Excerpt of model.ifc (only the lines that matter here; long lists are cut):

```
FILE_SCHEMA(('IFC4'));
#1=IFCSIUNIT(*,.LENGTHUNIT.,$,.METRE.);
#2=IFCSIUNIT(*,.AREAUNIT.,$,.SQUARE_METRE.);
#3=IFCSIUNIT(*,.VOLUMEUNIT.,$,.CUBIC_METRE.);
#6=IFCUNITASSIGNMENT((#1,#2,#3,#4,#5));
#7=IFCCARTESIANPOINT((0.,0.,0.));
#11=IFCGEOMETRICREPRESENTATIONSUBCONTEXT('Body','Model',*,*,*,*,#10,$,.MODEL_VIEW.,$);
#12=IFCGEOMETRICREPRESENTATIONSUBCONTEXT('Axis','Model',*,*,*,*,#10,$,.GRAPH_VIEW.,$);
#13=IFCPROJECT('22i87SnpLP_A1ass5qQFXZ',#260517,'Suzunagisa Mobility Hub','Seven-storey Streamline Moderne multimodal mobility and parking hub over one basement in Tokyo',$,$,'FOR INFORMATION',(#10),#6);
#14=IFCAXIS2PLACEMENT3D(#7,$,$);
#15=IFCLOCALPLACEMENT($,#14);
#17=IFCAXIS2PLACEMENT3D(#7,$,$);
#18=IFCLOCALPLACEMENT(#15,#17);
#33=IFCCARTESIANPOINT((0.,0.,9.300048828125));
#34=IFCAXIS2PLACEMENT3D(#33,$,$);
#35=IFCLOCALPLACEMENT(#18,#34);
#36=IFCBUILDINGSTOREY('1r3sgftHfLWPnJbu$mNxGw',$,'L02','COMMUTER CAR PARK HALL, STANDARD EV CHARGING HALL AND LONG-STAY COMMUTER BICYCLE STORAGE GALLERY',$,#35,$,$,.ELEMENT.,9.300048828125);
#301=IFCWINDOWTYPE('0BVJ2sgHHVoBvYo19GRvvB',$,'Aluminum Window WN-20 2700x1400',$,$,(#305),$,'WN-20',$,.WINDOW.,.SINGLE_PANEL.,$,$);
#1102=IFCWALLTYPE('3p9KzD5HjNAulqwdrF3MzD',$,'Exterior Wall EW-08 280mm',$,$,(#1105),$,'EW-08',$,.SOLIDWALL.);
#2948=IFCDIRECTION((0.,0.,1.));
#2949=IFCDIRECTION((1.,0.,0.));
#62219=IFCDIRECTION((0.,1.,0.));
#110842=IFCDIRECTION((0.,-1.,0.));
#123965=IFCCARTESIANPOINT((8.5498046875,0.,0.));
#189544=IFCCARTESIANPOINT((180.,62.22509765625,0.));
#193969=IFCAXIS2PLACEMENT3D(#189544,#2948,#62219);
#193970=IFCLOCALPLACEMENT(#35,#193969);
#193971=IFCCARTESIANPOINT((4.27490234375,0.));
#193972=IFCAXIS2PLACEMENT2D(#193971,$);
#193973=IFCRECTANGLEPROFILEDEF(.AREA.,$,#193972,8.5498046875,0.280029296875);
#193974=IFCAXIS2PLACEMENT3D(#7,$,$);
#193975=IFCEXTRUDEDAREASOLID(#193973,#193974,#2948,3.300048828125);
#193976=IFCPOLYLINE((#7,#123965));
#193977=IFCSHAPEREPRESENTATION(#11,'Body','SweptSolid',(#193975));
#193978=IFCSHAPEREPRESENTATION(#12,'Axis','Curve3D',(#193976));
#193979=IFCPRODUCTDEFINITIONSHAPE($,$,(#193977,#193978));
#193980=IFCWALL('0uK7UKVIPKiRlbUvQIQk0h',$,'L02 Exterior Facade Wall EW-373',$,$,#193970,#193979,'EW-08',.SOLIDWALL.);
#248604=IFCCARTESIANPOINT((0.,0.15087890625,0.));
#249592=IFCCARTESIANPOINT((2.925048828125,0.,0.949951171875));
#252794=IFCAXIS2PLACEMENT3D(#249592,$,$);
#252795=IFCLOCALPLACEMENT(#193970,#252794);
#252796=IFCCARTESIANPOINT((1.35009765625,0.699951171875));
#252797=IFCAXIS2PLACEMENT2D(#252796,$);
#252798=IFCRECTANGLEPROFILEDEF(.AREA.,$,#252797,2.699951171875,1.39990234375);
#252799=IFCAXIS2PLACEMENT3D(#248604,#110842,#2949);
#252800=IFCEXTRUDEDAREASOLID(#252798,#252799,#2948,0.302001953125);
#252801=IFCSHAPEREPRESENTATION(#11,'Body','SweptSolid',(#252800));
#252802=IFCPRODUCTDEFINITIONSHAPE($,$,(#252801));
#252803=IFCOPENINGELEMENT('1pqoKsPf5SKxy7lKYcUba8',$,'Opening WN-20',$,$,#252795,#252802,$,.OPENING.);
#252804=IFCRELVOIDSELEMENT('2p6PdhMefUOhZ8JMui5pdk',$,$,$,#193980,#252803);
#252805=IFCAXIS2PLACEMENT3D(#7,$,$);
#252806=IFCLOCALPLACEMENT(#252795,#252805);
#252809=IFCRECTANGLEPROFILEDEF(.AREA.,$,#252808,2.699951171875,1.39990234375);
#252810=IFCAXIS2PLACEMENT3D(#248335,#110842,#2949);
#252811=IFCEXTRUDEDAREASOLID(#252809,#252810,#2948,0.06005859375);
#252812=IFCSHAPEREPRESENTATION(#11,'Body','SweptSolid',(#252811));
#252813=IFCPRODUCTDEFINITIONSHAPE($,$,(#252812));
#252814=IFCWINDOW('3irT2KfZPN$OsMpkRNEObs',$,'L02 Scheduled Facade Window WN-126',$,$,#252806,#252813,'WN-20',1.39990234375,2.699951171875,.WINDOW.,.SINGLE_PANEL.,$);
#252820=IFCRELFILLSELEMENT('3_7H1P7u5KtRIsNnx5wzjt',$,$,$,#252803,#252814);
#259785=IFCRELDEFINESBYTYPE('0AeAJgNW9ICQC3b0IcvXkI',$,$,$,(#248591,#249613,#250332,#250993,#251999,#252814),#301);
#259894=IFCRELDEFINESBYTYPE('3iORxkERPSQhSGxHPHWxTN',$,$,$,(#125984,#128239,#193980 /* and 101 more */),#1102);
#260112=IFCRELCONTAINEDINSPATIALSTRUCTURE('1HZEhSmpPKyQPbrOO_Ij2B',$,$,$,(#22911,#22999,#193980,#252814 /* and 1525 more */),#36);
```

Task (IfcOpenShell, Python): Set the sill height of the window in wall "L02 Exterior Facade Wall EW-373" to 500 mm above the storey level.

```python
import numpy as np
import ifcopenshell
import ifcopenshell.api.geometry
import ifcopenshell.geom
import ifcopenshell.util.element
import ifcopenshell.util.placement
import ifcopenshell.util.shape
import ifcopenshell.util.unit

model = ifcopenshell.open("model.ifc")
unit_scale = ifcopenshell.util.unit.calculate_unit_scale(model)

window = model.by_guid("3irT2KfZPN$OsMpkRNEObs")
opening = window.FillsVoids[0].RelatingOpeningElement
storey = ifcopenshell.util.element.get_container(window, ifc_class="IfcBuildingStorey")
level = ifcopenshell.util.placement.get_local_placement(storey.ObjectPlacement)[2, 3]

# The opening's origin need not be at the sill, so measure its lowest point.
shape = ifcopenshell.geom.create_shape(ifcopenshell.geom.settings(), opening)
bottom = ifcopenshell.util.shape.get_shape_bottom_elevation(shape, shape.geometry) / unit_scale
dz = level + 0.5 - bottom

shift = np.array([0.0, 0.0, dz])
# The window is placed relative to its opening, so it follows when the opening moves.
matrix = ifcopenshell.util.placement.get_local_placement(opening.ObjectPlacement)
matrix[:3, 3] += shift
ifcopenshell.api.geometry.edit_object_placement(
    model, product=opening, matrix=matrix, is_si=False, should_transform_children=True
)

print(f"moved by {dz * unit_scale:+.3f} m")

model.write("model-out.ifc")
```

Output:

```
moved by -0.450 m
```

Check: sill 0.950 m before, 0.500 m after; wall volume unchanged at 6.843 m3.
